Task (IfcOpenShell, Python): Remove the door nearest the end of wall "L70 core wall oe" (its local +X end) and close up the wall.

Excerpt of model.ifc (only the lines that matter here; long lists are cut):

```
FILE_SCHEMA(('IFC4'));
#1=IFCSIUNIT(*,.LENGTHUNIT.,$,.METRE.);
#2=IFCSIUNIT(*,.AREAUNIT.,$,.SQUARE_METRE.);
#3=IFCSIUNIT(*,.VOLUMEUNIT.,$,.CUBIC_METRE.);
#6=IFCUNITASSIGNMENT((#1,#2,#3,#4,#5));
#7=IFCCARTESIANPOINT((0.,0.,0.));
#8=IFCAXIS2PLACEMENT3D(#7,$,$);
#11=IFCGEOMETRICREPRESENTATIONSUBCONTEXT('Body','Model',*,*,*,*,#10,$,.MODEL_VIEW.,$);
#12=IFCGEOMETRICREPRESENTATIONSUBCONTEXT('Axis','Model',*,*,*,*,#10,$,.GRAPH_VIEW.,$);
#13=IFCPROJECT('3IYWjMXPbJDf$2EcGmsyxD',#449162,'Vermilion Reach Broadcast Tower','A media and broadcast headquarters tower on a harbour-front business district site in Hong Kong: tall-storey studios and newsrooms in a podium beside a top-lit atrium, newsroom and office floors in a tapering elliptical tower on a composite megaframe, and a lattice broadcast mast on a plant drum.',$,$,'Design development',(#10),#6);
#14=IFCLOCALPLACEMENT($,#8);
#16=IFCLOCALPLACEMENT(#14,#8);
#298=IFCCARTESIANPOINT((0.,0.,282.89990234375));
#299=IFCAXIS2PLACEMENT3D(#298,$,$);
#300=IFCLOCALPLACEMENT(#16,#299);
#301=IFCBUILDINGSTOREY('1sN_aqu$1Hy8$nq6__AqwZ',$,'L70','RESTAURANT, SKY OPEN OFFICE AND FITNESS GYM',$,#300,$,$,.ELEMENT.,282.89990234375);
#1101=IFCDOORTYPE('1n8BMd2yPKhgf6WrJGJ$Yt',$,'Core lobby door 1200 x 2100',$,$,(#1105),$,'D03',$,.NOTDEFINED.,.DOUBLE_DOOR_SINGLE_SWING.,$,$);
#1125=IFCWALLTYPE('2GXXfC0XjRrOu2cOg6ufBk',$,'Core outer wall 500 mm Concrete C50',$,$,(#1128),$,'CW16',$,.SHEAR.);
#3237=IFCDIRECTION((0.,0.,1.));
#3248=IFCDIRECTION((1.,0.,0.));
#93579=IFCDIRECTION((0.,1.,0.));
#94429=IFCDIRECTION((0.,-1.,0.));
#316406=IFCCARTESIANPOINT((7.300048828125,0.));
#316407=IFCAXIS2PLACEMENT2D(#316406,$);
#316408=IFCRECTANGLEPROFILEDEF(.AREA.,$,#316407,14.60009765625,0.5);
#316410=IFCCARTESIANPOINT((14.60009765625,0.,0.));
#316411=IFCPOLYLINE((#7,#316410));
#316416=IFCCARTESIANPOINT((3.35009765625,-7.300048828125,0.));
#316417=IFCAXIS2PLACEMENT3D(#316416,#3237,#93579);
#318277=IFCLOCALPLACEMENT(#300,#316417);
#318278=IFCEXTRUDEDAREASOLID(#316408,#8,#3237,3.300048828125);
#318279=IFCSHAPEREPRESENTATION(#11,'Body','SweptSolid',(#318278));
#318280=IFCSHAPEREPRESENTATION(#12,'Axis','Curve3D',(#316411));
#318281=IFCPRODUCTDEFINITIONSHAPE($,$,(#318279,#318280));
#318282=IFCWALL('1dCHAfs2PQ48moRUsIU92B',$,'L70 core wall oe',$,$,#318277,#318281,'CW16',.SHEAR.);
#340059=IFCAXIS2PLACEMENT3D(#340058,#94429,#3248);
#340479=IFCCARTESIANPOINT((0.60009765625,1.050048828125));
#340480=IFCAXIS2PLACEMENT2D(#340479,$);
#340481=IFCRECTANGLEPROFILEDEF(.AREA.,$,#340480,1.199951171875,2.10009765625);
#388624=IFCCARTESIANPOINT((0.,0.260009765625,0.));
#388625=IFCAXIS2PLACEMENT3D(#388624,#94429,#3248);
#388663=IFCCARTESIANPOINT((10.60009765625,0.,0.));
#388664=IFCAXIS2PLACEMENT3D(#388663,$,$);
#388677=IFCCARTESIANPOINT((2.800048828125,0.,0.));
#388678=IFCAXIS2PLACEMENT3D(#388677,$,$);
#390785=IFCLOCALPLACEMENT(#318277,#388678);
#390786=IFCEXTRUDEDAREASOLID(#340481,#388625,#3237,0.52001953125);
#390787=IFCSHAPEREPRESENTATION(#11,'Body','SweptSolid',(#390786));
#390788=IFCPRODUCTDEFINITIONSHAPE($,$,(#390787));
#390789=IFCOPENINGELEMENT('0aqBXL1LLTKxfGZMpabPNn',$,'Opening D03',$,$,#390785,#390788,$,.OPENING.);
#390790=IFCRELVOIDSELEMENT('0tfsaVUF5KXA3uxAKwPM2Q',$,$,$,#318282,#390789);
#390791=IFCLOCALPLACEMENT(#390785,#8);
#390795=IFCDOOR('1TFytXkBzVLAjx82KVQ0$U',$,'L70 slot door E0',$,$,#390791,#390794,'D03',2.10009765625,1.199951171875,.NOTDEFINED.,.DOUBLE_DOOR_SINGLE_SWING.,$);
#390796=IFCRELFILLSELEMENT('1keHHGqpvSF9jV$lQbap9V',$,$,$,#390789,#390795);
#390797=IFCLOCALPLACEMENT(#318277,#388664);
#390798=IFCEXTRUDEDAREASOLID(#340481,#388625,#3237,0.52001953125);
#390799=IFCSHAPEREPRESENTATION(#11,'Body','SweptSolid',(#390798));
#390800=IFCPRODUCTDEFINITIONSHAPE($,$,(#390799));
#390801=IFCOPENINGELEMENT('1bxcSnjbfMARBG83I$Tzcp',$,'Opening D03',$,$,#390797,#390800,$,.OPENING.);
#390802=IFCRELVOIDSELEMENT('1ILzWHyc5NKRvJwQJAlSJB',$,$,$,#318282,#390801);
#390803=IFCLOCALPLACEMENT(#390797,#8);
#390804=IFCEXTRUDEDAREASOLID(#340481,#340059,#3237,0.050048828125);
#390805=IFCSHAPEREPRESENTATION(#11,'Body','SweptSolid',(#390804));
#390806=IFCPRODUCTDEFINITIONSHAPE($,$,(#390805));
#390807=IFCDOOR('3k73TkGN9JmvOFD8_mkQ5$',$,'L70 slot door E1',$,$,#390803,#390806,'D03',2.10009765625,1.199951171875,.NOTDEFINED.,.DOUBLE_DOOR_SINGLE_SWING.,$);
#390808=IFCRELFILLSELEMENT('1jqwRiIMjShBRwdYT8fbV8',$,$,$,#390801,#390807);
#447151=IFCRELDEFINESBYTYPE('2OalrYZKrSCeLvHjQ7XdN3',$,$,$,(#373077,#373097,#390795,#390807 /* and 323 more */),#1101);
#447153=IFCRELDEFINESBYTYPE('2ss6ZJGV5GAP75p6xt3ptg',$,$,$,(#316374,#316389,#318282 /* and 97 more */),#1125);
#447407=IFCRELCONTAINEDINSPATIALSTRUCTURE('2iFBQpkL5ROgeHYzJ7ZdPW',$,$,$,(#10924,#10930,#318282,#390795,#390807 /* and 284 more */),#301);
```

```python
import ifcopenshell
import ifcopenshell.api.feature
import ifcopenshell.api.root
import ifcopenshell.geom
import ifcopenshell.util.shape

model = ifcopenshell.open("model.ifc")
settings = ifcopenshell.geom.settings()


def volume(element):
    """Net volume in cubic metres, openings subtracted."""
    shape = ifcopenshell.geom.create_shape(settings, element)
    return ifcopenshell.util.shape.get_volume(shape.geometry)


door = model.by_guid("3k73TkGN9JmvOFD8_mkQ5$")
opening = door.FillsVoids[0].RelatingOpeningElement
wall = opening.VoidsElements[0].RelatingBuildingElement
before = volume(wall)

ifcopenshell.api.root.remove_product(model, product=door)
ifcopenshell.api.feature.remove_feature(model, feature=opening)

after = volume(wall)

print(f"wall volume {before:.3f} -> {after:.3f} m3")

model.write("model_rev.ifc")
```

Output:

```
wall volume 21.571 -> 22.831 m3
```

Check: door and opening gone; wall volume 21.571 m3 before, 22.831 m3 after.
